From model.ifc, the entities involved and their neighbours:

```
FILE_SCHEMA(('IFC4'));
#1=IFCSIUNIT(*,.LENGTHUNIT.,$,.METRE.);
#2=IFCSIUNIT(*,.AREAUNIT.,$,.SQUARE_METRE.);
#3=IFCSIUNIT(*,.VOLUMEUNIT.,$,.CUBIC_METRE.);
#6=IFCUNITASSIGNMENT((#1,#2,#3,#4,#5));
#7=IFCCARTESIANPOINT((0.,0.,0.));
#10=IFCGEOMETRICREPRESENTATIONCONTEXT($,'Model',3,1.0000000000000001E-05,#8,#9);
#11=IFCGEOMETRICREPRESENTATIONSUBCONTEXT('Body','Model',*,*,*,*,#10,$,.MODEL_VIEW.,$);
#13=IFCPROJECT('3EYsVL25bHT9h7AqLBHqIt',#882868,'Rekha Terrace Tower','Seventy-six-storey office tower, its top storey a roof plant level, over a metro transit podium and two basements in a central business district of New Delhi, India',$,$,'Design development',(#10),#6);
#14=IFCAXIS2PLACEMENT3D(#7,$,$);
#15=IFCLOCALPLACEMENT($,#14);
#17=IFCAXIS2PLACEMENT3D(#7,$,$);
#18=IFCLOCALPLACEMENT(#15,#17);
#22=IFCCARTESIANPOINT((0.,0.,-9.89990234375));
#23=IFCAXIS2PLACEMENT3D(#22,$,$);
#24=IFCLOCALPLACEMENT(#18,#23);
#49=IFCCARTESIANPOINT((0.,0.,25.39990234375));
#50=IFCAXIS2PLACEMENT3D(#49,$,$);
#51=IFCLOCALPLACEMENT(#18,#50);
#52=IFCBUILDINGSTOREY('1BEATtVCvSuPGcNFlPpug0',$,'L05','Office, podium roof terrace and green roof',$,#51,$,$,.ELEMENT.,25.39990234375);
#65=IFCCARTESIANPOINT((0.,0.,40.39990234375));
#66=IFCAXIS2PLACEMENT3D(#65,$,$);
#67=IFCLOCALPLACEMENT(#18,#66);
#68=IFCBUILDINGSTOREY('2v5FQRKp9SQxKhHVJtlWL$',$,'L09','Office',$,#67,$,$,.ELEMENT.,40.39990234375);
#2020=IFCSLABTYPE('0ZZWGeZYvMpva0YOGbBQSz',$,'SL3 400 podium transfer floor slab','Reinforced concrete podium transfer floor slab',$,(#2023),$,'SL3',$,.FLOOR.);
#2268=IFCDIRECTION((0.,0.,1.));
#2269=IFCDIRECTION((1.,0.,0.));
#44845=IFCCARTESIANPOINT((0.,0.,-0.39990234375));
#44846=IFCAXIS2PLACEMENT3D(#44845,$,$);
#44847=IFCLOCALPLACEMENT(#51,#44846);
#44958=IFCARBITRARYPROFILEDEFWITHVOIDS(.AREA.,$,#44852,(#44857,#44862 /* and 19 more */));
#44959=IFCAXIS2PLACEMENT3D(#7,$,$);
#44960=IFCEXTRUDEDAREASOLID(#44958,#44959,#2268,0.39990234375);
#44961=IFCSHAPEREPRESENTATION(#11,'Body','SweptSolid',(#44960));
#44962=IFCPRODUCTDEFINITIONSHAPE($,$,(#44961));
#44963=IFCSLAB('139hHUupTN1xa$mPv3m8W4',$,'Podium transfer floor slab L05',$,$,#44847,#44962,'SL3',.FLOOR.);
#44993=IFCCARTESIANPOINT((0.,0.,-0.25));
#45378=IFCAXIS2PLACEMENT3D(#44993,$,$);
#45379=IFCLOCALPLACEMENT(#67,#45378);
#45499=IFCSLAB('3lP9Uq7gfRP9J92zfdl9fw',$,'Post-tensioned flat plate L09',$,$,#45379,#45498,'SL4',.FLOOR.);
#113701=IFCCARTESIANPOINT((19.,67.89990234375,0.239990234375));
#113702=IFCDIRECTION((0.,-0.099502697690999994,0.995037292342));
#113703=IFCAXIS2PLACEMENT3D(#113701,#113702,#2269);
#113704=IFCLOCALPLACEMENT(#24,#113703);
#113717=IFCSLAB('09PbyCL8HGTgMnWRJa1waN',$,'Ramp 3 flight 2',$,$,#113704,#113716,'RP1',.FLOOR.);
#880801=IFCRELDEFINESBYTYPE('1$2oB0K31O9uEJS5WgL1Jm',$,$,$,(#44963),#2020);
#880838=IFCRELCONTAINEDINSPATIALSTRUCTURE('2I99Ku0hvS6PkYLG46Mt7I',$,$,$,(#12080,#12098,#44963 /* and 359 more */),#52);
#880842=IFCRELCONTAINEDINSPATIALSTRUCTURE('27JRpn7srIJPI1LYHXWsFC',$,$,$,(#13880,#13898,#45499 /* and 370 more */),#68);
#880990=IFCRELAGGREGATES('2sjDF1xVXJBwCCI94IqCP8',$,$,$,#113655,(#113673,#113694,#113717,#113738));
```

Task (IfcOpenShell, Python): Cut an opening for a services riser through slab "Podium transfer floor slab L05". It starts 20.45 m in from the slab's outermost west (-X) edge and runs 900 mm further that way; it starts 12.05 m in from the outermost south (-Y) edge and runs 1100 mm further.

```python
import numpy as np
import ifcopenshell
import ifcopenshell.api.feature
import ifcopenshell.api.geometry
import ifcopenshell.api.root
import ifcopenshell.geom
import ifcopenshell.util.placement
import ifcopenshell.util.representation
import ifcopenshell.util.shape
import ifcopenshell.util.unit

model = ifcopenshell.open("model.ifc")
unit_scale = ifcopenshell.util.unit.calculate_unit_scale(model)
settings = ifcopenshell.geom.settings()


def volume(element):
    """Net volume in cubic metres, openings subtracted."""
    shape = ifcopenshell.geom.create_shape(settings, element)
    return ifcopenshell.util.shape.get_volume(shape.geometry)


slab = model.by_guid("139hHUupTN1xa$mPv3m8W4")
before = volume(slab)

# Extent in the slab's own axes, in metres. The edges named are its -X and -Y sides.
slab_shape = ifcopenshell.geom.create_shape(settings, slab)
vertices = ifcopenshell.util.shape.get_vertices(slab_shape.geometry)
x_min, y_min, bottom = vertices.min(axis=0)
top = vertices[:, 2].max()

opening = ifcopenshell.api.root.create_entity(model, ifc_class="IfcOpeningElement", name="Services riser opening", predefined_type="OPENING")
context = ifcopenshell.util.representation.get_context(model, "Model", "Body", "MODEL_VIEW")
width, depth = 0.9, 1.1
outline = [(0.0, 0.0), (width, 0.0), (width, depth), (0.0, depth), (0.0, 0.0)]
# Overshoot both faces by 50 mm so the cut is clean.
shape = ifcopenshell.api.geometry.add_slab_representation(
    model, context=context, depth=top - bottom + 0.1, polyline=outline
)
ifcopenshell.api.geometry.assign_representation(model, product=opening, representation=shape)

matrix = ifcopenshell.util.placement.get_local_placement(slab.ObjectPlacement)
matrix[:, 3] = matrix @ np.append(np.array([x_min + 20.45, y_min + 12.05, bottom - 0.05]) / unit_scale, 1.0)
ifcopenshell.api.geometry.edit_object_placement(model, product=opening, matrix=matrix, is_si=False)
ifcopenshell.api.feature.add_feature(model, feature=opening, element=slab)

after = volume(slab)

print(f"slab volume {before:.3f} -> {after:.3f} m3")

model.write("model_updated.ifc")
```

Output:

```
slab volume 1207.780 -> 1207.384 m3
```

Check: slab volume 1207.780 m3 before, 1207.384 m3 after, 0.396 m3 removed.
